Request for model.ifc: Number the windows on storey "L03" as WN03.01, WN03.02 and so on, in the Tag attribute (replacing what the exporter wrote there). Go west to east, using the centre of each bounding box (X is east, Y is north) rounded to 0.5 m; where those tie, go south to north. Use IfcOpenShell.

First a look at what the model holds.

```python
import ifcopenshell
import ifcopenshell.util.element
import ifcopenshell.util.placement

model = ifcopenshell.open("model.ifc")
print(model.schema)
storey = next(s for s in model.by_type("IfcBuildingStorey") if s.Name == "L03")
windows = [e for e in ifcopenshell.util.element.get_decomposition(storey) if e.is_a("IfcWindow")]
for e in sorted(windows, key=lambda e: e.id()):
    origin = ifcopenshell.util.placement.get_local_placement(e.ObjectPlacement)[:3, 3]
    print(e.id(), e.Tag, e.Name, origin.round(2) + 0.0, sep=" | ")
```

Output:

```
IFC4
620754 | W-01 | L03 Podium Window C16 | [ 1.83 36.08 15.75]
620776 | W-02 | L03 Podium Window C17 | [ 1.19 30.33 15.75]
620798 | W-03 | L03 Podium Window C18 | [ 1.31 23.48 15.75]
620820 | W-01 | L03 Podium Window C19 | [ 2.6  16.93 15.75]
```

```python
import ifcopenshell
import ifcopenshell.geom
import ifcopenshell.util.element
import ifcopenshell.util.shape

model = ifcopenshell.open("model.ifc")
settings = ifcopenshell.geom.settings()
settings.set("use-world-coords", True)


def centre(element):
    shape = ifcopenshell.geom.create_shape(settings, element)
    return ifcopenshell.util.shape.get_bbox_centroid(shape.geometry)


storey = next(s for s in model.by_type("IfcBuildingStorey") if s.Name == "L03")
windows = [e for e in ifcopenshell.util.element.get_decomposition(storey) if e.is_a("IfcWindow")]

# Insertion points can sit at a corner or the storey origin, so sort by the geometry (in metres).
centres = {e: centre(e) for e in windows}
windows.sort(key=lambda e: (round(centres[e][0] / 0.5), centres[e][1]))

for i, e in enumerate(windows, start=1):
    number = f"WN03.{i:02d}"
    e.Tag = number
    print(e.id(), number)

model.write("model_updated.ifc")
```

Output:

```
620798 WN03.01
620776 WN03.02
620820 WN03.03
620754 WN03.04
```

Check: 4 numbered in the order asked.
